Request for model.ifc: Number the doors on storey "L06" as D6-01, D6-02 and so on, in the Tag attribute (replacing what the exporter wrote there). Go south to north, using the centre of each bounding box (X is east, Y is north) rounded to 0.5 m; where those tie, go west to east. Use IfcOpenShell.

First a look at what the model holds.

```python
import ifcopenshell
import ifcopenshell.util.element
import ifcopenshell.util.placement

model = ifcopenshell.open("model.ifc")
print(model.schema)
storey = next(s for s in model.by_type("IfcBuildingStorey") if s.Name == "L06")
doors = [e for e in ifcopenshell.util.element.get_decomposition(storey) if e.is_a("IfcDoor")]
for e in sorted(doors, key=lambda e: e.id()):
    origin = ifcopenshell.util.placement.get_local_placement(e.ObjectPlacement)[:3, 3]
    print(e.id(), e.Tag, e.Name, origin.round(2) + 0.0, sep=" | ")
```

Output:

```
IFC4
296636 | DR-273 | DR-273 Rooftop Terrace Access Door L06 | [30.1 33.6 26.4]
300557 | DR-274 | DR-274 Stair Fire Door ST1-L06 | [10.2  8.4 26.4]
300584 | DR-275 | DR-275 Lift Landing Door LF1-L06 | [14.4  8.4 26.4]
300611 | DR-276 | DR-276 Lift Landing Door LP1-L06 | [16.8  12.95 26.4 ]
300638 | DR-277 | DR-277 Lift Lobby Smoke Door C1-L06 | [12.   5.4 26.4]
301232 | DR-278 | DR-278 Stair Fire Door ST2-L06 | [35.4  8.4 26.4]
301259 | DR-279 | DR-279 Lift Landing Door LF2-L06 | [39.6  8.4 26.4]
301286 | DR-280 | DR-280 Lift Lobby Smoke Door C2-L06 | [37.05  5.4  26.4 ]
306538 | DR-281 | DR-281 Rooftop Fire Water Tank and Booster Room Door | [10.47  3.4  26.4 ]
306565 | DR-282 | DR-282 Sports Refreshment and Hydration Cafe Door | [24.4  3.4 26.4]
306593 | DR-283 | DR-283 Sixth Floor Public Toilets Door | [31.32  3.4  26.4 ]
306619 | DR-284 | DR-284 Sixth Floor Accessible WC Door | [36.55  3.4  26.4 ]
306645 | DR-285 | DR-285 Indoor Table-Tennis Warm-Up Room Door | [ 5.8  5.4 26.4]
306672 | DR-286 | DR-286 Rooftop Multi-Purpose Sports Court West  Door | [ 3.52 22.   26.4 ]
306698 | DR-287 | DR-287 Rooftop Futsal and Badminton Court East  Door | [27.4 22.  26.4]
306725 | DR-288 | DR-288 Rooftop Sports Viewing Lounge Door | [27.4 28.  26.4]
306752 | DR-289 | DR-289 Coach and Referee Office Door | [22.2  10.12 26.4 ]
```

```python
import ifcopenshell
import ifcopenshell.geom
import ifcopenshell.util.element
import ifcopenshell.util.shape

model = ifcopenshell.open("model.ifc")
settings = ifcopenshell.geom.settings()
settings.set("use-world-coords", True)


def centre(element):
    shape = ifcopenshell.geom.create_shape(settings, element)
    return ifcopenshell.util.shape.get_bbox_centroid(shape.geometry)


storey = next(s for s in model.by_type("IfcBuildingStorey") if s.Name == "L06")
doors = [e for e in ifcopenshell.util.element.get_decomposition(storey) if e.is_a("IfcDoor")]

# Insertion points can sit at a corner or the storey origin, so sort by the geometry (in metres).
centres = {e: centre(e) for e in doors}
doors.sort(key=lambda e: (round(centres[e][1] / 0.5), centres[e][0]))

for i, e in enumerate(doors, start=1):
    number = f"D6-{i:02d}"
    e.Tag = number
    print(e.id(), number)

model.write("model_edited.ifc")
```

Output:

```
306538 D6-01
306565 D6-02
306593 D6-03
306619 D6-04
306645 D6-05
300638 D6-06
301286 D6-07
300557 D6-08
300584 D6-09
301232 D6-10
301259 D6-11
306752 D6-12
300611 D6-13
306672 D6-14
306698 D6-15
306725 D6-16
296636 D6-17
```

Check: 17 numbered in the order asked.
